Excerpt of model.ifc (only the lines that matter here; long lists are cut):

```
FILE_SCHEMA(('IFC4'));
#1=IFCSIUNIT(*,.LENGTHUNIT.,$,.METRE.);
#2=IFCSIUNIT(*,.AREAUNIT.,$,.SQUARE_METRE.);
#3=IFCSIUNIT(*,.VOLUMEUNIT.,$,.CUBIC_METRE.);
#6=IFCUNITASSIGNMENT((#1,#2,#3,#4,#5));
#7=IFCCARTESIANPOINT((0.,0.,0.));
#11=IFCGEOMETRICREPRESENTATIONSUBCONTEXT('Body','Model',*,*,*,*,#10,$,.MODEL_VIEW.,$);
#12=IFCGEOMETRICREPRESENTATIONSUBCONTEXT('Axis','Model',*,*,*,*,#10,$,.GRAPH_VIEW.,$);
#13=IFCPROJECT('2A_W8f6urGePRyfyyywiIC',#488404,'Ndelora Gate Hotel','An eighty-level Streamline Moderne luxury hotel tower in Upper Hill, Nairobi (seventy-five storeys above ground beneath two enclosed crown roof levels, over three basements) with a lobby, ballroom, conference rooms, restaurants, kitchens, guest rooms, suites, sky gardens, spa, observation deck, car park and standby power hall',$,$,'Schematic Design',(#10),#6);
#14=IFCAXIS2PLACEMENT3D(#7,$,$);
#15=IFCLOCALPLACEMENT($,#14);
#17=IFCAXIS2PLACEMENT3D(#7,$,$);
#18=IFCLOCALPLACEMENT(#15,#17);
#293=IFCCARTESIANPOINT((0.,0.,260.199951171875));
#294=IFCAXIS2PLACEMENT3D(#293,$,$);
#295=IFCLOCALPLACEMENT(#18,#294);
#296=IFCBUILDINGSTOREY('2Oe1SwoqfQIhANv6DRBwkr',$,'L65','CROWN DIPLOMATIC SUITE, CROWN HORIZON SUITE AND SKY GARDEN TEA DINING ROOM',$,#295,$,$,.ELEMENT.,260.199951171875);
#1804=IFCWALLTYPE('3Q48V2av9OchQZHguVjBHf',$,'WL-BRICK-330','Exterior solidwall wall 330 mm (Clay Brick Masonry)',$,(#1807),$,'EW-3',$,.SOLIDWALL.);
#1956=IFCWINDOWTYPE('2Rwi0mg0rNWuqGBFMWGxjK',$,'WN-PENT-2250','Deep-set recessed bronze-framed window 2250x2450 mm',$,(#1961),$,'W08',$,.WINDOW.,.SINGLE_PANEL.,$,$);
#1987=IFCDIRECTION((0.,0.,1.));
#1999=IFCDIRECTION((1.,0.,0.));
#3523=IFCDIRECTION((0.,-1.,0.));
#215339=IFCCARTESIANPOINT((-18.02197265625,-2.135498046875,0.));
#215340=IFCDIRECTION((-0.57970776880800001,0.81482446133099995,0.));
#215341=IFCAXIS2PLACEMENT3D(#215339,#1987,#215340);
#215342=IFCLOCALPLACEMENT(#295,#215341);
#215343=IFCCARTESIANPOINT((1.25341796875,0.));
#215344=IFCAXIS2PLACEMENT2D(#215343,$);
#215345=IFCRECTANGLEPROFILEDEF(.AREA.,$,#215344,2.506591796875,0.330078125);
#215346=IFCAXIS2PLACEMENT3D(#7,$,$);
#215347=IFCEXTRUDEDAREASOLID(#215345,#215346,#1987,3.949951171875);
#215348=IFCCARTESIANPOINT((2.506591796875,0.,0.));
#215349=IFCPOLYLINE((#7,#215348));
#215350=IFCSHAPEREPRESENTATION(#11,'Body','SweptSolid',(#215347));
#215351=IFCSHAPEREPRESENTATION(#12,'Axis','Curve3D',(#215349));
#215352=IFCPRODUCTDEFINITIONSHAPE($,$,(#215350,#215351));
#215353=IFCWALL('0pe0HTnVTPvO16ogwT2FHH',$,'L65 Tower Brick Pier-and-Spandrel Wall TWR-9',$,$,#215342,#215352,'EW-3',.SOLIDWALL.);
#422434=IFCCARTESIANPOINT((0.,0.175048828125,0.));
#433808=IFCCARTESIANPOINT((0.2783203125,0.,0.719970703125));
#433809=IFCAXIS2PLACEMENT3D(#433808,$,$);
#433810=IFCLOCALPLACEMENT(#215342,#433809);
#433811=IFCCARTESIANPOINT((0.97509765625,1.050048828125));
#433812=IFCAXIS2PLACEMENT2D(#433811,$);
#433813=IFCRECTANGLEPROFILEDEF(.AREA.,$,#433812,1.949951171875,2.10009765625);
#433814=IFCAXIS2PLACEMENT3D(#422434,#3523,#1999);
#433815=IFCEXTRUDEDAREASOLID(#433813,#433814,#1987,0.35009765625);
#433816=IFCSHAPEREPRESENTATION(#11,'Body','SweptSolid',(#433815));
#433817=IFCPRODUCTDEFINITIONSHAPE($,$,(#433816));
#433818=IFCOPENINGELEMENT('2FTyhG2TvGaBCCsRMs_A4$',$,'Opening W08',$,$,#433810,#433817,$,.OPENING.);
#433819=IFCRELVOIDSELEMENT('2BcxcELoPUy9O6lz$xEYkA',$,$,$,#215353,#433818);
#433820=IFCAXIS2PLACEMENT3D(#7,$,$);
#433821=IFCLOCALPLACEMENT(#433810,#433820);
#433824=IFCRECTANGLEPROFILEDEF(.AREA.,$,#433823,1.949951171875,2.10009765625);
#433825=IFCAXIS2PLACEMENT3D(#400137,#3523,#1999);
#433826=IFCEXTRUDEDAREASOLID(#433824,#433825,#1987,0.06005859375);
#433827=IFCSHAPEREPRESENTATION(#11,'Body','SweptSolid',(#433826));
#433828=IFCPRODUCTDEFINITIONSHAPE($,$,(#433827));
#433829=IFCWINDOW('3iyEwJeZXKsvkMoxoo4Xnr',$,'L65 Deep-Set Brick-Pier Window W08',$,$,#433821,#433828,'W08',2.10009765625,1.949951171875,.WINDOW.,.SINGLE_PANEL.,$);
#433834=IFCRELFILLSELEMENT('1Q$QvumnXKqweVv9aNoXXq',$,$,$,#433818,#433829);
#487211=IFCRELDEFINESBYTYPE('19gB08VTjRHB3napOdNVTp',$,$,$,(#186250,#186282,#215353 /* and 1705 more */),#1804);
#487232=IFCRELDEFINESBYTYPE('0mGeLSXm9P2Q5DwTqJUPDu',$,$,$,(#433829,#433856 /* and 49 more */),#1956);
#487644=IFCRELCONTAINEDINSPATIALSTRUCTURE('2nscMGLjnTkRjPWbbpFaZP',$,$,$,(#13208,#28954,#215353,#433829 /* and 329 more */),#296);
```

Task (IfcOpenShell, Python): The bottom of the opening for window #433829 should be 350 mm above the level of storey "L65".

```python
import numpy as np
import ifcopenshell
import ifcopenshell.api.geometry
import ifcopenshell.geom
import ifcopenshell.util.element
import ifcopenshell.util.placement
import ifcopenshell.util.shape
import ifcopenshell.util.unit

model = ifcopenshell.open("model.ifc")
unit_scale = ifcopenshell.util.unit.calculate_unit_scale(model)

window = model.by_id(433829)
opening = window.FillsVoids[0].RelatingOpeningElement
storey = ifcopenshell.util.element.get_container(window, ifc_class="IfcBuildingStorey")
level = ifcopenshell.util.placement.get_local_placement(storey.ObjectPlacement)[2, 3]

# The opening's origin need not be at the sill, so measure its lowest point.
shape = ifcopenshell.geom.create_shape(ifcopenshell.geom.settings(), opening)
bottom = ifcopenshell.util.shape.get_shape_bottom_elevation(shape, shape.geometry) / unit_scale
dz = level + 0.35 - bottom

shift = np.array([0.0, 0.0, dz])
# The window is placed relative to its opening, so it follows when the opening moves.
matrix = ifcopenshell.util.placement.get_local_placement(opening.ObjectPlacement)
matrix[:3, 3] += shift
ifcopenshell.api.geometry.edit_object_placement(
    model, product=opening, matrix=matrix, is_si=False, should_transform_children=True
)

print(f"moved by {dz * unit_scale:+.3f} m")

model.write("model_updated.ifc")
```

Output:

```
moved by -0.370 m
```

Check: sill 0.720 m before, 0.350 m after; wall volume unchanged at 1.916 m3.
